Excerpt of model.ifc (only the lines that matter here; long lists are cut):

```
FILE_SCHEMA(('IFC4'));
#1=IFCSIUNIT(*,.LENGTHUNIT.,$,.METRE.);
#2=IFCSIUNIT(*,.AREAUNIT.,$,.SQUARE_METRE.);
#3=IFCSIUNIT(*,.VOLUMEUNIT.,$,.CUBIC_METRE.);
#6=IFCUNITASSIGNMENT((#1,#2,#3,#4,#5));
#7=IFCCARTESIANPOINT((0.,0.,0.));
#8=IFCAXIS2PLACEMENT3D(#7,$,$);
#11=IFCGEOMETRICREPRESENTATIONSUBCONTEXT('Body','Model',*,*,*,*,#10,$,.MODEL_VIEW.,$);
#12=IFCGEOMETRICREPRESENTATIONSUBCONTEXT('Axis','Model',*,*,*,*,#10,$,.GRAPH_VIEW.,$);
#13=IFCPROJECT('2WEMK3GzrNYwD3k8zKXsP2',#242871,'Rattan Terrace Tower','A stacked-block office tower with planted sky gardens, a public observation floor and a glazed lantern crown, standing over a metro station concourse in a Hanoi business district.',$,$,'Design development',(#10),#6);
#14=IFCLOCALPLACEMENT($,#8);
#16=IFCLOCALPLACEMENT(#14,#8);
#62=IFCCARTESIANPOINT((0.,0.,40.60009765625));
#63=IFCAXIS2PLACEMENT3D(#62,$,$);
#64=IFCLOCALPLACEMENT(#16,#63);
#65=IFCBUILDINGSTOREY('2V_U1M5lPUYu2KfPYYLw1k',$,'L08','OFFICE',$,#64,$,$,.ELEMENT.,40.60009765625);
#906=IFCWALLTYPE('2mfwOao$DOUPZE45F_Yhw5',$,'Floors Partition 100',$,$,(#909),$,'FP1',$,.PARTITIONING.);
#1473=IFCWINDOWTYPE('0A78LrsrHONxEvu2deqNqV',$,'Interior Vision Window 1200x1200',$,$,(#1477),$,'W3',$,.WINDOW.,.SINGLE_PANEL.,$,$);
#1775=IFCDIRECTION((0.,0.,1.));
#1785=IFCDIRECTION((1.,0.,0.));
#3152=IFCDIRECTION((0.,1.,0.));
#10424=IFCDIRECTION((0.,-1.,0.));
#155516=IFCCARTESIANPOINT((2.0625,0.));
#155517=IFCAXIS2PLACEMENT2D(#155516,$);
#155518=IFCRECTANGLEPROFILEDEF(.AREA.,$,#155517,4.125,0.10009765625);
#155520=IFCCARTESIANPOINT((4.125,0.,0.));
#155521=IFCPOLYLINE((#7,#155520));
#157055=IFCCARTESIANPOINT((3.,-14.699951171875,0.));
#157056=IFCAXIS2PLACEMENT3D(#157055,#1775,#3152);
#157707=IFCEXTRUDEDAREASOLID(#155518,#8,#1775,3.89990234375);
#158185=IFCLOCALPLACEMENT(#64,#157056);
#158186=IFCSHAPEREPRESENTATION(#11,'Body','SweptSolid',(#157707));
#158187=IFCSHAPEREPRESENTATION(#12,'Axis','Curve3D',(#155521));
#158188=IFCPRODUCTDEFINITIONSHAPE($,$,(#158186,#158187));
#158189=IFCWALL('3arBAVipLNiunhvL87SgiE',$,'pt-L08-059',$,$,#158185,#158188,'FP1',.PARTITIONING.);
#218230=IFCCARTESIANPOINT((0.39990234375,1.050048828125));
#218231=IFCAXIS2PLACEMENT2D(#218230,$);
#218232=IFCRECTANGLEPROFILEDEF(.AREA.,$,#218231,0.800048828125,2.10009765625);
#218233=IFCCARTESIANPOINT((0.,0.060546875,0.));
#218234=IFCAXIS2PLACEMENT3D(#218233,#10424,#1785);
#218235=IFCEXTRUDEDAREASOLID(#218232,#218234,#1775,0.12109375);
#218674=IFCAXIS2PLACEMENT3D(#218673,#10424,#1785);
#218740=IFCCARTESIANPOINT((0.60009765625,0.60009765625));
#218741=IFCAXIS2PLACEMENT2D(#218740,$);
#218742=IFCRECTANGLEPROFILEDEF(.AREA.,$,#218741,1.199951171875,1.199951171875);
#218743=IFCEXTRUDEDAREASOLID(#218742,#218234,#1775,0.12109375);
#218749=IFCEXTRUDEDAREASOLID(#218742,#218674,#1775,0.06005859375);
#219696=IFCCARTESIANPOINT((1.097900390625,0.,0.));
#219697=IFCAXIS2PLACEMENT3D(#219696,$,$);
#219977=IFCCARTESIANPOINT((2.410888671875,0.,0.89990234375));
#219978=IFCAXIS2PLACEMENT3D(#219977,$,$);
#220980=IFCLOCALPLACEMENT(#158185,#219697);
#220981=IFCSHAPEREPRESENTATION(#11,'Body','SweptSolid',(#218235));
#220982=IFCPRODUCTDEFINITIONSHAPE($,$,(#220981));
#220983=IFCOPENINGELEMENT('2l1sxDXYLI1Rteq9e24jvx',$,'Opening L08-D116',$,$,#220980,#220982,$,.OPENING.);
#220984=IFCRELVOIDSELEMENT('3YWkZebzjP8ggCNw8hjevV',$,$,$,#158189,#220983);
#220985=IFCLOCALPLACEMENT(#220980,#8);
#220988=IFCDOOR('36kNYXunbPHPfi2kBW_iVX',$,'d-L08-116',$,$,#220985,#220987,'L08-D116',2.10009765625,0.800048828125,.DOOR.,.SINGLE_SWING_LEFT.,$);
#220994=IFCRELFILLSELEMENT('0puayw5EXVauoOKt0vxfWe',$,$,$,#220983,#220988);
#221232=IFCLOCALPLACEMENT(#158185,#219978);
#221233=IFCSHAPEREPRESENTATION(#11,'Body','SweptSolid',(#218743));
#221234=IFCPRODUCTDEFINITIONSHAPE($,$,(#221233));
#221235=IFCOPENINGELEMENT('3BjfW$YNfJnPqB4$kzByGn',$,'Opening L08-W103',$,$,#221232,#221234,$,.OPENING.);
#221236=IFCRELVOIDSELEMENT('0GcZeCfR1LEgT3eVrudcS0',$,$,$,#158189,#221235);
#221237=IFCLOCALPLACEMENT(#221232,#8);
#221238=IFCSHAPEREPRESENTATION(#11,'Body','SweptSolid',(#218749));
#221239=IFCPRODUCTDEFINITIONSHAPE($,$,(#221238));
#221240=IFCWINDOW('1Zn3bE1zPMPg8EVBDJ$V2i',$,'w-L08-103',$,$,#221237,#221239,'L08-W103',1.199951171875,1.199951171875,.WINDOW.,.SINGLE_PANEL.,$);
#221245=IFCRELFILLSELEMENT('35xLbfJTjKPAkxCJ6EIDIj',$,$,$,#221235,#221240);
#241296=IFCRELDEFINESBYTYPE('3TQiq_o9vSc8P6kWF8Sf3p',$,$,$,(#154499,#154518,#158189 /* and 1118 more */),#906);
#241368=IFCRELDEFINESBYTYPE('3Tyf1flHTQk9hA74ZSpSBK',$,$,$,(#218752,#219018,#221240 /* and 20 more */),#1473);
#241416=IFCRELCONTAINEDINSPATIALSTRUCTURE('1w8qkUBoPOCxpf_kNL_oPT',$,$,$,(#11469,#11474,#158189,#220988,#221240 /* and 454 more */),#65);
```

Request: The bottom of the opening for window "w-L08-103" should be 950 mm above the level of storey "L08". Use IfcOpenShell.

```python
import numpy as np
import ifcopenshell
import ifcopenshell.api.geometry
import ifcopenshell.geom
import ifcopenshell.util.element
import ifcopenshell.util.placement
import ifcopenshell.util.shape
import ifcopenshell.util.unit

model = ifcopenshell.open("model.ifc")
unit_scale = ifcopenshell.util.unit.calculate_unit_scale(model)

window = model.by_id(221240)
opening = window.FillsVoids[0].RelatingOpeningElement
storey = ifcopenshell.util.element.get_container(window, ifc_class="IfcBuildingStorey")
level = ifcopenshell.util.placement.get_local_placement(storey.ObjectPlacement)[2, 3]

# The opening's origin need not be at the sill, so measure its lowest point.
shape = ifcopenshell.geom.create_shape(ifcopenshell.geom.settings(), opening)
bottom = ifcopenshell.util.shape.get_shape_bottom_elevation(shape, shape.geometry) / unit_scale
dz = level + 0.95 / unit_scale - bottom

shift = np.array([0.0, 0.0, dz])
# The window is placed relative to its opening, so it follows when the opening moves.
matrix = ifcopenshell.util.placement.get_local_placement(opening.ObjectPlacement)
matrix[:3, 3] += shift
ifcopenshell.api.geometry.edit_object_placement(
    model, product=opening, matrix=matrix, is_si=False, should_transform_children=True
)

print(f"moved by {dz * unit_scale:+.3f} m")

model.write("model_edited.ifc")
```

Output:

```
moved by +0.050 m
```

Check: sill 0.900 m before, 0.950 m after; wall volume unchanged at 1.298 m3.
